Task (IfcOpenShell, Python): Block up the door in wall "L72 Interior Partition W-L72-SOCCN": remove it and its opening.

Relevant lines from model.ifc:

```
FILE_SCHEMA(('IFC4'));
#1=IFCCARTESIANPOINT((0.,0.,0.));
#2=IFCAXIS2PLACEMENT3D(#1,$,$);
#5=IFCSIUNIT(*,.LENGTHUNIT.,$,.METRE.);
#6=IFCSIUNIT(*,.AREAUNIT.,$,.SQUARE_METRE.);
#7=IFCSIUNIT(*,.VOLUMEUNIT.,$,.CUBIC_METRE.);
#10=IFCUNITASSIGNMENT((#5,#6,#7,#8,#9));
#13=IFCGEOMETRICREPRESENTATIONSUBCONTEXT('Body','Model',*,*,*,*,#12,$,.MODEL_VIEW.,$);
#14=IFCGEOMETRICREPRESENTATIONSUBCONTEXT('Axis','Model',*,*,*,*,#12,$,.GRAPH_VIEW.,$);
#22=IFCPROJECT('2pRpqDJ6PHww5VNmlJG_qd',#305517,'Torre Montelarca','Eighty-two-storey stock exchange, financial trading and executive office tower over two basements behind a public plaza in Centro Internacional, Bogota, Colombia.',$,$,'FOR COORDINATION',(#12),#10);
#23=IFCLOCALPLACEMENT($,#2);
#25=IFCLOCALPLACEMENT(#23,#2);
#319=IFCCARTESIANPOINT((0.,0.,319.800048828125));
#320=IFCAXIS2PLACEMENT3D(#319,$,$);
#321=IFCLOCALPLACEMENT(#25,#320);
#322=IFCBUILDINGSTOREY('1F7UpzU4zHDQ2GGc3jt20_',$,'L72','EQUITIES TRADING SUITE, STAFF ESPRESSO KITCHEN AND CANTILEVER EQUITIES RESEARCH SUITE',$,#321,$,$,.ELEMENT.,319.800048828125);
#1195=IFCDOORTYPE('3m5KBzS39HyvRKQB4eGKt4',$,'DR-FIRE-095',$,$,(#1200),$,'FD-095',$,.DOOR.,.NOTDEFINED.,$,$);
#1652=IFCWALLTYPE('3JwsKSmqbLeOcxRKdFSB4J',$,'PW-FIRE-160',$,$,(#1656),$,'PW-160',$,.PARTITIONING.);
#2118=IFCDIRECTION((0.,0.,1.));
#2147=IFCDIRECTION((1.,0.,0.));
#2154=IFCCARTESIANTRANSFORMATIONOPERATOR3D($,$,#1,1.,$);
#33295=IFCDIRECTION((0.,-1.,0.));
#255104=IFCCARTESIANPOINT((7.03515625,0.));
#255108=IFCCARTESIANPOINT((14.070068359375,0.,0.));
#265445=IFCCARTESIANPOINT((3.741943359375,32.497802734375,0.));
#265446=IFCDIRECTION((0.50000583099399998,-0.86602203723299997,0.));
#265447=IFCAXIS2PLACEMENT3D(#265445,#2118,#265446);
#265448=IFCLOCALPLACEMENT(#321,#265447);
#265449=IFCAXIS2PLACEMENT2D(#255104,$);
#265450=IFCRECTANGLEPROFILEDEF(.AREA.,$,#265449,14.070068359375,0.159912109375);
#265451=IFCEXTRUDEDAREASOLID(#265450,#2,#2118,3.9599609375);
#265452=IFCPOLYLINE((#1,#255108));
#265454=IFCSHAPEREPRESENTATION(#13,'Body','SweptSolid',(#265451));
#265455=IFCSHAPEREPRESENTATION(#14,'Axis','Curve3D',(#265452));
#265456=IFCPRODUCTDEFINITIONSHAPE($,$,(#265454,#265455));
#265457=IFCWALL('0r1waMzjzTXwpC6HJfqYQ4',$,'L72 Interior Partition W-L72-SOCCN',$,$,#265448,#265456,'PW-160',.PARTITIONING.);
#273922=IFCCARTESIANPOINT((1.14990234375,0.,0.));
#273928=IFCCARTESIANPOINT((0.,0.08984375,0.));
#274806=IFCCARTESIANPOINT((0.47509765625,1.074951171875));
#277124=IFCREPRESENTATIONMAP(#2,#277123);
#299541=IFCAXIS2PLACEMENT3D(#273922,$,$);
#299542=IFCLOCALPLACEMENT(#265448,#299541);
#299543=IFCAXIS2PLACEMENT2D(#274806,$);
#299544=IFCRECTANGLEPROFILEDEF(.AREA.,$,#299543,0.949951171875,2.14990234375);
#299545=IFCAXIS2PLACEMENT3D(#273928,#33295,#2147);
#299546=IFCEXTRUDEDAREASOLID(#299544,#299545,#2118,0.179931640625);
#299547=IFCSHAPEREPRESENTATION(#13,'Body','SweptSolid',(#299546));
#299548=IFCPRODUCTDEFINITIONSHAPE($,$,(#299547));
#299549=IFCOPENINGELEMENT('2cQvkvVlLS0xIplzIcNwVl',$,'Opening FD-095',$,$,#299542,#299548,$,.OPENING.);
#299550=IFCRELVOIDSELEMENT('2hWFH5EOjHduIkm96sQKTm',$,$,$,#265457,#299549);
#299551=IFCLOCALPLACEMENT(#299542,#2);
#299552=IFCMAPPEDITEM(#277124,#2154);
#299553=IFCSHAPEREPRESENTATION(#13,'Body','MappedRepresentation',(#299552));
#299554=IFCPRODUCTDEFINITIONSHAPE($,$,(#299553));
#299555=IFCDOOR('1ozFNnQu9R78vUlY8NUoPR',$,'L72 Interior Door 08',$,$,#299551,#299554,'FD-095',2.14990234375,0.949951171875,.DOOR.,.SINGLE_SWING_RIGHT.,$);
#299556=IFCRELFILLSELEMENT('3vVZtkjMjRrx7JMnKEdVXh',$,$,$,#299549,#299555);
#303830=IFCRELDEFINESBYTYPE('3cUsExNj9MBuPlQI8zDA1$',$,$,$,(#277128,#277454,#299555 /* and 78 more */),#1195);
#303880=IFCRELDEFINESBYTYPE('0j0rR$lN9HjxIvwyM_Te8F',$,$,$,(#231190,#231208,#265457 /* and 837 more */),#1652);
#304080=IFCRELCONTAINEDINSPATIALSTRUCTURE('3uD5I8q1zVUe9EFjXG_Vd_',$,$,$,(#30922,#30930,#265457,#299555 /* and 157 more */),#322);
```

```python
import ifcopenshell
import ifcopenshell.api.feature
import ifcopenshell.api.root
import ifcopenshell.geom
import ifcopenshell.util.shape

model = ifcopenshell.open("model.ifc")
settings = ifcopenshell.geom.settings()


def volume(element):
    """Net volume in cubic metres, openings subtracted."""
    shape = ifcopenshell.geom.create_shape(settings, element)
    return ifcopenshell.util.shape.get_volume(shape.geometry)


door = model.by_id(299555)
opening = door.FillsVoids[0].RelatingOpeningElement
wall = opening.VoidsElements[0].RelatingBuildingElement
before = volume(wall)

ifcopenshell.api.root.remove_product(model, product=door)
ifcopenshell.api.feature.remove_feature(model, feature=opening)

after = volume(wall)

print(f"wall volume {before:.3f} -> {after:.3f} m3")

model.write("model_v2.ifc")
```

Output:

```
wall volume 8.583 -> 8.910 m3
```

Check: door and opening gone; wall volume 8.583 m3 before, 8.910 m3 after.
